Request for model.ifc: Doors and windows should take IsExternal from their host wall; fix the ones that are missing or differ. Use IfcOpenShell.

First a look at what the model holds.

```python
import ifcopenshell
import ifcopenshell.util.element

model = ifcopenshell.open("model.ifc")
print(model.schema)
seen = {}
for e in model.by_type("IfcDoor") + model.by_type("IfcWindow"):
    if not e.FillsVoids:
        continue
    host = e.FillsVoids[0].RelatingOpeningElement.VoidsElements[0].RelatingBuildingElement
    own = ifcopenshell.util.element.get_pset(e, f"Pset_{e.is_a()[3:].removesuffix('StandardCase')}Common", "IsExternal")
    wall = ifcopenshell.util.element.get_pset(host, "Pset_WallCommon", "IsExternal")
    seen[e.is_a(), own, wall] = seen.get((e.is_a(), own, wall), 0) + 1
for (cls, own, wall), count in sorted(seen.items(), key=str):
    print(count, cls, "IsExternal:", own, "| host wall:", wall)
```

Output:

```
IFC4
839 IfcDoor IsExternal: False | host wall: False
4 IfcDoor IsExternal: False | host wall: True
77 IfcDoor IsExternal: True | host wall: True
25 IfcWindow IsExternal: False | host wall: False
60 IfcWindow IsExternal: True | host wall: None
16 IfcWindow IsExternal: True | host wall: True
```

```python
import ifcopenshell
import ifcopenshell.api.pset
import ifcopenshell.util.element

model = ifcopenshell.open("model.ifc")

count = 0
for ifc_class, pset_name in (("IfcDoor", "Pset_DoorCommon"), ("IfcWindow", "Pset_WindowCommon")):
    for e in model.by_type(ifc_class):
        if not e.FillsVoids:
            continue
        host = e.FillsVoids[0].RelatingOpeningElement.VoidsElements[0].RelatingBuildingElement
        external = ifcopenshell.util.element.get_pset(host, "Pset_WallCommon", "IsExternal")
        if external is None or ifcopenshell.util.element.get_pset(e, pset_name, "IsExternal") == external:
            continue
        pset = ifcopenshell.api.pset.add_pset(model, product=e, name=pset_name)
        ifcopenshell.api.pset.edit_pset(model, pset=pset, properties={"IsExternal": external})
        count += 1

print(count, "updated")

model.write("model_updated.ifc")
```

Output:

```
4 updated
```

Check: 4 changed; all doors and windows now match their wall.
